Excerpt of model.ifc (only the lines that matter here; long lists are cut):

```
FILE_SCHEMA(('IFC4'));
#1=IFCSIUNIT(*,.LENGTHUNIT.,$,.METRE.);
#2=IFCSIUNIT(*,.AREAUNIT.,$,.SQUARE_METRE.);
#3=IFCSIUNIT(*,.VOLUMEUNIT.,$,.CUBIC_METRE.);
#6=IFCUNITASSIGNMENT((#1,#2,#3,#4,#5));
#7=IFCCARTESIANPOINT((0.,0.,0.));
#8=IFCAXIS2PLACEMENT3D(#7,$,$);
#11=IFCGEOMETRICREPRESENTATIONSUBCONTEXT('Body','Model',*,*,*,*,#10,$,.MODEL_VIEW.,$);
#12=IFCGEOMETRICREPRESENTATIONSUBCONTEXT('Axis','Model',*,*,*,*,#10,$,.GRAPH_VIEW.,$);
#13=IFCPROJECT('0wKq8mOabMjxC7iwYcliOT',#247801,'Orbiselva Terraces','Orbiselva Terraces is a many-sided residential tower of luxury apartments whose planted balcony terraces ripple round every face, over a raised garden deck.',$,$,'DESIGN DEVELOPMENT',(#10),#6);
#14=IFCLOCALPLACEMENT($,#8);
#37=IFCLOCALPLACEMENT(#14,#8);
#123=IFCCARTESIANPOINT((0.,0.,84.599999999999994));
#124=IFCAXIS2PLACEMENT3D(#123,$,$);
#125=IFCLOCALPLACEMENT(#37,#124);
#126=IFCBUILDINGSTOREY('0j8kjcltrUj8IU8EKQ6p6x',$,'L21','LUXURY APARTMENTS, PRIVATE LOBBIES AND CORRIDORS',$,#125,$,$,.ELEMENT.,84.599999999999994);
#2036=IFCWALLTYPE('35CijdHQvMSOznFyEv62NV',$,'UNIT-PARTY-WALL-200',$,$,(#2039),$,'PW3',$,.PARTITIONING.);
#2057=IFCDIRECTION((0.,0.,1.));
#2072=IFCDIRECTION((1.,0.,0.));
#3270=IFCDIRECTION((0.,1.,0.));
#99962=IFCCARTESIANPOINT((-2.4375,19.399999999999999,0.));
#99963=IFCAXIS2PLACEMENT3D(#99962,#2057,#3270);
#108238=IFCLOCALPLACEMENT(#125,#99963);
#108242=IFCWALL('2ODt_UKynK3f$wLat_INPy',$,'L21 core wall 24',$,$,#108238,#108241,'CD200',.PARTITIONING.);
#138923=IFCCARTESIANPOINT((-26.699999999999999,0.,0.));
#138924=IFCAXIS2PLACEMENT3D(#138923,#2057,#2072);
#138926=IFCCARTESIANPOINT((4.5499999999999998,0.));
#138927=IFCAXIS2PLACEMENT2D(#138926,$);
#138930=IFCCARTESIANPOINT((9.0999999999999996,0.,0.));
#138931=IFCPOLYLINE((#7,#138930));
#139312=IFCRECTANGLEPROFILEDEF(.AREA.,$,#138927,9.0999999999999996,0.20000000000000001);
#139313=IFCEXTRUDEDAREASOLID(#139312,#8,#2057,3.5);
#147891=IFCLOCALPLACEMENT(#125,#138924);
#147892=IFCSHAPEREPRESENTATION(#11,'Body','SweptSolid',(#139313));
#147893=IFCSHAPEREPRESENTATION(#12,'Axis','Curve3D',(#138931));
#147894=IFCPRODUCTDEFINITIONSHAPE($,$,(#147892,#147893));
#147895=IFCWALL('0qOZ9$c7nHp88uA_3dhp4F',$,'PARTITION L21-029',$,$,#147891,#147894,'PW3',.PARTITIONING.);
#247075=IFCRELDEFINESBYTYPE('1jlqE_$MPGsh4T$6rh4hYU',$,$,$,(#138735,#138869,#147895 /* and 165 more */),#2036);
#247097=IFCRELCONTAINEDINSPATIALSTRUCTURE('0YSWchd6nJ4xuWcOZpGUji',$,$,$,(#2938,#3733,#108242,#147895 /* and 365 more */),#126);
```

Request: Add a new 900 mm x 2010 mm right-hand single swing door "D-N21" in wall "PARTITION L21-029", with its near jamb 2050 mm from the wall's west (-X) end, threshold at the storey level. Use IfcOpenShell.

```python
import numpy as np
import ifcopenshell
import ifcopenshell.api.feature
import ifcopenshell.api.geometry
import ifcopenshell.api.root
import ifcopenshell.api.spatial
import ifcopenshell.geom
import ifcopenshell.util.element
import ifcopenshell.util.placement
import ifcopenshell.util.representation
import ifcopenshell.util.shape
import ifcopenshell.util.unit

model = ifcopenshell.open("model.ifc")
unit_scale = ifcopenshell.util.unit.calculate_unit_scale(model)
settings = ifcopenshell.geom.settings()


def volume(element):
    """Net volume in cubic metres, openings subtracted."""
    shape = ifcopenshell.geom.create_shape(settings, element)
    return ifcopenshell.util.shape.get_volume(shape.geometry)


wall = model.by_id(147895)
storey = ifcopenshell.util.element.get_container(wall, ifc_class="IfcBuildingStorey")
context = ifcopenshell.util.representation.get_context(model, "Model", "Body", "MODEL_VIEW")
before = volume(wall)

width, height, from_end, sill = 0.9, 2.01, 2.05, 0.0  # metres

# The wall runs along its own X axis, and the end named is its -X end.
wall_shape = ifcopenshell.geom.create_shape(settings, wall)
x, y, z = ifcopenshell.util.shape.get_vertices(wall_shape.geometry).T
start = x.min() + from_end
face, thickness = float(y.min()), float(y.max() - y.min())
wall_matrix = ifcopenshell.util.placement.get_local_placement(wall.ObjectPlacement)
level = ifcopenshell.util.placement.get_local_placement(storey.ObjectPlacement)[2, 3]


def in_wall(x, y):
    """Placement at x, y metres in the wall's axes, at sill height."""
    matrix = wall_matrix.copy()
    matrix[:, 3] = wall_matrix @ np.array([x / unit_scale, y / unit_scale, 0.0, 1.0])
    matrix[2, 3] = level + sill / unit_scale
    return matrix


# Opening: a box that overshoots both wall faces by 50 mm.
opening = ifcopenshell.api.root.create_entity(model, ifc_class="IfcOpeningElement", predefined_type="OPENING")
box = ifcopenshell.api.geometry.add_wall_representation(
    model, context=context, length=width, height=height, thickness=thickness + 0.1
)
ifcopenshell.api.geometry.assign_representation(model, product=opening, representation=box)
ifcopenshell.api.geometry.edit_object_placement(model, product=opening, matrix=in_wall(start, face - 0.05), is_si=False)
ifcopenshell.api.feature.add_feature(model, feature=opening, element=wall)

door = ifcopenshell.api.root.create_entity(model, ifc_class="IfcDoor", name="D-N21", predefined_type="DOOR")
door.OverallWidth, door.OverallHeight = width / unit_scale, height / unit_scale
door.OperationType = "SINGLE_SWING_RIGHT"
body = ifcopenshell.api.geometry.add_door_representation(
    model,
    context=context,
    overall_width=door.OverallWidth,
    overall_height=door.OverallHeight,
    operation_type="SINGLE_SWING_RIGHT",
    lining_properties={"LiningDepth": thickness / unit_scale, "ThresholdDepth": thickness / unit_scale},
)
ifcopenshell.api.geometry.assign_representation(model, product=door, representation=body)
ifcopenshell.api.spatial.assign_container(model, products=[door], relating_structure=storey)
ifcopenshell.api.feature.add_filling(model, opening=opening, element=door)

# The lining spans the wall, so the door starts at the wall face.
ifcopenshell.api.geometry.edit_object_placement(model, product=door, matrix=in_wall(start, face), is_si=False)

after = volume(wall)

print(f"wall volume {before:.3f} -> {after:.3f} m3")

model.write("model_v2.ifc")
```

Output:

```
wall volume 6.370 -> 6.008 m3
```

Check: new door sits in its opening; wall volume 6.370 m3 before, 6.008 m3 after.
